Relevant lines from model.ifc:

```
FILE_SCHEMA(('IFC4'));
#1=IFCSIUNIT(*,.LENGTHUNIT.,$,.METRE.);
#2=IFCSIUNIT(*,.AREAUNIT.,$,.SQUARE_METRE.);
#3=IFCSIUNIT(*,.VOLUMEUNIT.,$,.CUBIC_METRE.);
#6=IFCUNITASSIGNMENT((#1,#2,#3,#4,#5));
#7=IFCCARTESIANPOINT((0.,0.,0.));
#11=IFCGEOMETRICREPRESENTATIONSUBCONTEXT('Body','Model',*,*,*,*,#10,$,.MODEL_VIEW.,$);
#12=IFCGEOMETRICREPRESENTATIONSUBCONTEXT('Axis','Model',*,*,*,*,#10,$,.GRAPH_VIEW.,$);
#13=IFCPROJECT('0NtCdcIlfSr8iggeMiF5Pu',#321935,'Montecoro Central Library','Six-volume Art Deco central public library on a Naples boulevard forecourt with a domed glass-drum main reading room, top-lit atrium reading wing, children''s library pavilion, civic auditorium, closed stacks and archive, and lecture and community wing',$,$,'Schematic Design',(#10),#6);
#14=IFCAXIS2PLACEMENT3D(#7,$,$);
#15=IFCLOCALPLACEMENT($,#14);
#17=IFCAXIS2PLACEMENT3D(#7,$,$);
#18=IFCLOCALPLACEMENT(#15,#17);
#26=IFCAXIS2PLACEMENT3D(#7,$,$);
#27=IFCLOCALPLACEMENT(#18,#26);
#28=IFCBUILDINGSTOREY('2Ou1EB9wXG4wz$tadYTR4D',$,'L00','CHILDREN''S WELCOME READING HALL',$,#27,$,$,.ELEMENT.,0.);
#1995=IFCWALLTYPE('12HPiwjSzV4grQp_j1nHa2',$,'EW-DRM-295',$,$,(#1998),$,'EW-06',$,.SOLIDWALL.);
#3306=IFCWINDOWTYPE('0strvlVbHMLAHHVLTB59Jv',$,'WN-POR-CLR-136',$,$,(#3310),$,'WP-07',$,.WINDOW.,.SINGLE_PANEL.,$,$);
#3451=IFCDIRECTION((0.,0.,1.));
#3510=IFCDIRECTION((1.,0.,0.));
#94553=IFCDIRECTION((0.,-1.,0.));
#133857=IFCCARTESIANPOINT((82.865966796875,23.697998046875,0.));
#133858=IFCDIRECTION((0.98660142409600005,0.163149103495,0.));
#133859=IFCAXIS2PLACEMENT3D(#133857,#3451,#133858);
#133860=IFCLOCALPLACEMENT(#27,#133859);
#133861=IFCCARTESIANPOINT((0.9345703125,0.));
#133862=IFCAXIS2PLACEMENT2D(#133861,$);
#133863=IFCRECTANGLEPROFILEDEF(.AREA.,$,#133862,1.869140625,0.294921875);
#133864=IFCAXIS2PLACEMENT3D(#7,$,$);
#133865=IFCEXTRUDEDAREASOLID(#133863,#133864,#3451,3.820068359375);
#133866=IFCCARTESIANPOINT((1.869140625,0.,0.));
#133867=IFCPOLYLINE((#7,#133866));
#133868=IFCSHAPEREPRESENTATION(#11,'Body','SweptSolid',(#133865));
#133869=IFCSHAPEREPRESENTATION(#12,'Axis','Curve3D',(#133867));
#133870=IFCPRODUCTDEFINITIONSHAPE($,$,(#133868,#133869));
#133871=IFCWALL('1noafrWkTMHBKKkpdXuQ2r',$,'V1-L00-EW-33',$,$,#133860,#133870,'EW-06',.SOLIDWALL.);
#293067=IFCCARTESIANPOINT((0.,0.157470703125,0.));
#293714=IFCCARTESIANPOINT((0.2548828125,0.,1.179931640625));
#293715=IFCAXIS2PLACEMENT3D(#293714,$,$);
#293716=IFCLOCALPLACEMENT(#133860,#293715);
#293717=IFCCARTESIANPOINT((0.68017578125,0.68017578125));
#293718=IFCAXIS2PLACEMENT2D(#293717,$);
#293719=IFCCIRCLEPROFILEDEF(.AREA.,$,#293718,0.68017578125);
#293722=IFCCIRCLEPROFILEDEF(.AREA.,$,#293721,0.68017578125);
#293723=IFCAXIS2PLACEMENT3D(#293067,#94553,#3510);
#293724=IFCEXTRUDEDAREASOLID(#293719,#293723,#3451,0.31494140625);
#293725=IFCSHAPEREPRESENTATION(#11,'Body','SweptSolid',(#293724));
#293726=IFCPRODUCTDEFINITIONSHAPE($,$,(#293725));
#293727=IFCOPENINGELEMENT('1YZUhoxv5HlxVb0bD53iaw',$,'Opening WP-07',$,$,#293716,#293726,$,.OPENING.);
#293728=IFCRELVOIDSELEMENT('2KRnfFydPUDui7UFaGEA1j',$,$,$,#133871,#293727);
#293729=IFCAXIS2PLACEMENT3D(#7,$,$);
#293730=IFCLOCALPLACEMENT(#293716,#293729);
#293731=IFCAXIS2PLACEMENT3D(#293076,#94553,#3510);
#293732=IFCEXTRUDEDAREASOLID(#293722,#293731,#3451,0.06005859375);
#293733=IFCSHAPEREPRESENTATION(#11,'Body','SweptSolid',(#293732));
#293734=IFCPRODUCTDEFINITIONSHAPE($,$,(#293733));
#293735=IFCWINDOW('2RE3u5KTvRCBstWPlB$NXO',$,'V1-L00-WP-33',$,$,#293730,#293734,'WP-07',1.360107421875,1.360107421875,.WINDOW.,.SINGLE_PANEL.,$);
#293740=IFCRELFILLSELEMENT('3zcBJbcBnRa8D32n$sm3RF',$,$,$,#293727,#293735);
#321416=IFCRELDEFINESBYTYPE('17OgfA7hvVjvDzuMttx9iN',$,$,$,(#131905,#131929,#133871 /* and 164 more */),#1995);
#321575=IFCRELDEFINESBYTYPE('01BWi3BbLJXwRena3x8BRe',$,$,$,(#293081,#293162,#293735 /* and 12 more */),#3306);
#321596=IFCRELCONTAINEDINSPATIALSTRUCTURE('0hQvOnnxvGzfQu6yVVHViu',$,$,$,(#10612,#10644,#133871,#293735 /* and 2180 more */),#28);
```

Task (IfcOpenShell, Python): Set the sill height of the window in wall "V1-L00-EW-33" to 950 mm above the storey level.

```python
import numpy as np
import ifcopenshell
import ifcopenshell.api.geometry
import ifcopenshell.geom
import ifcopenshell.util.element
import ifcopenshell.util.placement
import ifcopenshell.util.shape
import ifcopenshell.util.unit

model = ifcopenshell.open("model.ifc")
unit_scale = ifcopenshell.util.unit.calculate_unit_scale(model)

window = model.by_guid("2RE3u5KTvRCBstWPlB$NXO")
opening = window.FillsVoids[0].RelatingOpeningElement
storey = ifcopenshell.util.element.get_container(window, ifc_class="IfcBuildingStorey")
level = ifcopenshell.util.placement.get_local_placement(storey.ObjectPlacement)[2, 3]

# The opening's origin need not be at the sill, so measure its lowest point.
shape = ifcopenshell.geom.create_shape(ifcopenshell.geom.settings(), opening)
bottom = ifcopenshell.util.shape.get_shape_bottom_elevation(shape, shape.geometry) / unit_scale
dz = level + 0.95 - bottom

shift = np.array([0.0, 0.0, dz])
# The window is placed relative to its opening, so it follows when the opening moves.
matrix = ifcopenshell.util.placement.get_local_placement(opening.ObjectPlacement)
matrix[:3, 3] += shift
ifcopenshell.api.geometry.edit_object_placement(
    model, product=opening, matrix=matrix, is_si=False, should_transform_children=True
)

print(f"moved by {dz * unit_scale:+.3f} m")

model.write("model_rev.ifc")
```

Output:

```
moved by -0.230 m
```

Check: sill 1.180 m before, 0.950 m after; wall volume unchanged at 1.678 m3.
